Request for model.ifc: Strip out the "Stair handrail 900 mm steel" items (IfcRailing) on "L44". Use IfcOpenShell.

First a look at what the model holds.

```python
import ifcopenshell
import ifcopenshell.util.element

model = ifcopenshell.open("model.ifc")
print(model.schema)
storey = next(s for s in model.by_type("IfcBuildingStorey") if s.Name == "L44")
railings = [e for e in ifcopenshell.util.element.get_decomposition(storey) if e.is_a("IfcRailing")]
seen = {}
for e in railings:
    element_type = ifcopenshell.util.element.get_type(e)
    name = element_type.Name if element_type not in (None, e) else None
    seen[name] = seen.get(name, 0) + 1
for name, count in sorted(seen.items(), key=str):
    print(count, "x", name)
```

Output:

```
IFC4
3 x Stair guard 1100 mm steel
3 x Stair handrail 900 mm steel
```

```python
import ifcopenshell
import ifcopenshell.api.root
import ifcopenshell.util.element

model = ifcopenshell.open("model.ifc")

storey = next(s for s in model.by_type("IfcBuildingStorey") if s.Name == "L44")
railings = [e for e in ifcopenshell.util.element.get_decomposition(storey) if e.is_a("IfcRailing")]
targets = [e for e in railings if (t := ifcopenshell.util.element.get_type(e)) not in (None, e) and t.Name == "Stair handrail 900 mm steel"]

for e in targets:
    ifcopenshell.api.root.remove_product(model, product=e)
print(len(targets), "removed")

model.write("model-out.ifc")
```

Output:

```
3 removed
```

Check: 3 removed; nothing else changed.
